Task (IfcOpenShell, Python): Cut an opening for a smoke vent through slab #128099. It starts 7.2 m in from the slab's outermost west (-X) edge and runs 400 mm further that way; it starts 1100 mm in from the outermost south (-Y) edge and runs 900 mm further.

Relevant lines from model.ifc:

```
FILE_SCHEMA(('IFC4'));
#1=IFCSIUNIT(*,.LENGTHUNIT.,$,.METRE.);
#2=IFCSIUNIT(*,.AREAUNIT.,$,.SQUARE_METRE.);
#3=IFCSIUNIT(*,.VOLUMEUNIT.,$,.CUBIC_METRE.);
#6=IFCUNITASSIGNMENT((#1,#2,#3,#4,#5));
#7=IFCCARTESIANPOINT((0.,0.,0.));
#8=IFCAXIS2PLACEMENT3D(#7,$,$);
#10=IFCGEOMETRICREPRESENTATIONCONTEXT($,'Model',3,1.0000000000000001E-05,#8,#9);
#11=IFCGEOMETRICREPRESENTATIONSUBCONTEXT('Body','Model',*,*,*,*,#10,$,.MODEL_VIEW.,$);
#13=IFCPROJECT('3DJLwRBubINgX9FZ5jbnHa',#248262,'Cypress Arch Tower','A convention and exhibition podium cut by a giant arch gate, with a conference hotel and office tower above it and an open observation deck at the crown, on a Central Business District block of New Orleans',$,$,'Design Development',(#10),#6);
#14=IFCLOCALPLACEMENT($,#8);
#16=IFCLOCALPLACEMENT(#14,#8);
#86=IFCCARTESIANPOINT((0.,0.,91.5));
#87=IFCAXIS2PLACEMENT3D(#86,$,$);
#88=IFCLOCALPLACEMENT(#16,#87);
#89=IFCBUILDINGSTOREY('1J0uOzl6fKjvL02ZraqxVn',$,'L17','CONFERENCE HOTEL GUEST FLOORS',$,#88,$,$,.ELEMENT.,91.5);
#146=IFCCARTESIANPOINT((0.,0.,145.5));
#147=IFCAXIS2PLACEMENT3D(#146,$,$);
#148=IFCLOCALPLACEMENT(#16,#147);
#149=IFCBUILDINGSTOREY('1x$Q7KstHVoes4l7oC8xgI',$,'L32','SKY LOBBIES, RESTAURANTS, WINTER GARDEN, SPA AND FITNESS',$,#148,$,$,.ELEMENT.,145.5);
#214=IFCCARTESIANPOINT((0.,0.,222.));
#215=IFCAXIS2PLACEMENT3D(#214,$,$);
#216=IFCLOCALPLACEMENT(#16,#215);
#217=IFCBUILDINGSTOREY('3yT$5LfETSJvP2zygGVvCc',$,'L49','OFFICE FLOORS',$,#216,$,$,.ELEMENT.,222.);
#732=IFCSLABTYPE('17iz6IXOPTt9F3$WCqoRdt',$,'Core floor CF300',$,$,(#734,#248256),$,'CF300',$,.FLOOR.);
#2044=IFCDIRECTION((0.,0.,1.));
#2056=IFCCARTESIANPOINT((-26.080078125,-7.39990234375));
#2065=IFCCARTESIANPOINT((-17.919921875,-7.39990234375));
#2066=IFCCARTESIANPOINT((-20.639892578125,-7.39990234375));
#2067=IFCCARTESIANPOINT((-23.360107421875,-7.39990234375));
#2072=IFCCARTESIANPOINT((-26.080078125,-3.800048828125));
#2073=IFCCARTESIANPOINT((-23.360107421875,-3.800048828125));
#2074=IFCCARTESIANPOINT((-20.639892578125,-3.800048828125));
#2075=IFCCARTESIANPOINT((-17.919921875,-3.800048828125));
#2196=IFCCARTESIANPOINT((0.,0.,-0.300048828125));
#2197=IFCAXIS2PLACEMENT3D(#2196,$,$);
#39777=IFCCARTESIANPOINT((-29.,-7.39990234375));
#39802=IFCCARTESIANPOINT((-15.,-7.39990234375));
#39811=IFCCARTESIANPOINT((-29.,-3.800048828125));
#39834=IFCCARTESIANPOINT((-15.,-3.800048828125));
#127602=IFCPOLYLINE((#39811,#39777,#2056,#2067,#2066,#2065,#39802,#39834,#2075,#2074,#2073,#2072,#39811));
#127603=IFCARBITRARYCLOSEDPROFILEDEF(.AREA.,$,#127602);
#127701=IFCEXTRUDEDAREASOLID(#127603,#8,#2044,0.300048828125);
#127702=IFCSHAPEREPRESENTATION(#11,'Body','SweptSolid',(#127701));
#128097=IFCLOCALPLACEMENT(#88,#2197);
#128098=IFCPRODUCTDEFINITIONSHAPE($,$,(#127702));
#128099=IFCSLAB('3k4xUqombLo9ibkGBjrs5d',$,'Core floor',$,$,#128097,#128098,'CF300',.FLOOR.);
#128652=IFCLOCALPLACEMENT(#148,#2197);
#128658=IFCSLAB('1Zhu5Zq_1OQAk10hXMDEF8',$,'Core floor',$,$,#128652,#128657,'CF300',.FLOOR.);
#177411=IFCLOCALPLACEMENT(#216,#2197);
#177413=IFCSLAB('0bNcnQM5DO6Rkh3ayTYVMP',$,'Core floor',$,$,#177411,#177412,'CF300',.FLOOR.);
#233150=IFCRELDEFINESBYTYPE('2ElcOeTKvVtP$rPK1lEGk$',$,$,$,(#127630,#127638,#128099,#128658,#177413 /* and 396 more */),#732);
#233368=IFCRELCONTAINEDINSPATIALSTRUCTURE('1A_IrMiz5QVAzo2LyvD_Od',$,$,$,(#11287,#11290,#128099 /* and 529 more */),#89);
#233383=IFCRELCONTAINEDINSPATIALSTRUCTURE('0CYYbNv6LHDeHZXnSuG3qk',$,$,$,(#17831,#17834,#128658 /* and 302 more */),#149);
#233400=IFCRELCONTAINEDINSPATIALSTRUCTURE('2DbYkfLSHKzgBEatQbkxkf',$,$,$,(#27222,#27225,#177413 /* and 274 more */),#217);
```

```python
import numpy as np
import ifcopenshell
import ifcopenshell.api.feature
import ifcopenshell.api.geometry
import ifcopenshell.api.root
import ifcopenshell.geom
import ifcopenshell.util.placement
import ifcopenshell.util.representation
import ifcopenshell.util.shape
import ifcopenshell.util.unit

model = ifcopenshell.open("model.ifc")
unit_scale = ifcopenshell.util.unit.calculate_unit_scale(model)
settings = ifcopenshell.geom.settings()


def volume(element):
    """Net volume in cubic metres, openings subtracted."""
    shape = ifcopenshell.geom.create_shape(settings, element)
    return ifcopenshell.util.shape.get_volume(shape.geometry)


slab = model.by_guid("3k4xUqombLo9ibkGBjrs5d")
before = volume(slab)

# Extent in the slab's own axes, in metres. The edges named are its -X and -Y sides.
slab_shape = ifcopenshell.geom.create_shape(settings, slab)
vertices = ifcopenshell.util.shape.get_vertices(slab_shape.geometry)
x_min, y_min, bottom = vertices.min(axis=0)
top = vertices[:, 2].max()

opening = ifcopenshell.api.root.create_entity(model, ifc_class="IfcOpeningElement", name="Smoke vent opening", predefined_type="OPENING")
context = ifcopenshell.util.representation.get_context(model, "Model", "Body", "MODEL_VIEW")
width, depth = 0.4, 0.9
outline = [(0.0, 0.0), (width, 0.0), (width, depth), (0.0, depth), (0.0, 0.0)]
# Overshoot both faces by 50 mm so the cut is clean.
shape = ifcopenshell.api.geometry.add_slab_representation(
    model, context=context, depth=top - bottom + 0.1, polyline=outline
)
ifcopenshell.api.geometry.assign_representation(model, product=opening, representation=shape)

matrix = ifcopenshell.util.placement.get_local_placement(slab.ObjectPlacement)
matrix[:, 3] = matrix @ np.append(np.array([x_min + 7.2, y_min + 1.1, bottom - 0.05]) / unit_scale, 1.0)
ifcopenshell.api.geometry.edit_object_placement(model, product=opening, matrix=matrix, is_si=False)
ifcopenshell.api.feature.add_feature(model, feature=opening, element=slab)

after = volume(slab)

print(f"slab volume {before:.3f} -> {after:.3f} m3")

model.write("model_updated.ifc")
```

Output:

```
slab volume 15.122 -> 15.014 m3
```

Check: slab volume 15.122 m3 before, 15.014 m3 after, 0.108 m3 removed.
